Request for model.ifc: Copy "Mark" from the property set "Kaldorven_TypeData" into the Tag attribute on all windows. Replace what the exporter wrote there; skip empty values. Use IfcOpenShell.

First a look at what the model holds.

```python
import ifcopenshell
import ifcopenshell.util.element

model = ifcopenshell.open("model.ifc")
print(model.schema)
windows = model.by_type("IfcWindow")
print(len(windows), "windows")
for e in windows[:8]:
    source = ifcopenshell.util.element.get_pset(e, "Kaldorven_TypeData", "Mark")
    target = e.Tag
    print(e.id(), repr(source), repr(target), sep=" | ")
```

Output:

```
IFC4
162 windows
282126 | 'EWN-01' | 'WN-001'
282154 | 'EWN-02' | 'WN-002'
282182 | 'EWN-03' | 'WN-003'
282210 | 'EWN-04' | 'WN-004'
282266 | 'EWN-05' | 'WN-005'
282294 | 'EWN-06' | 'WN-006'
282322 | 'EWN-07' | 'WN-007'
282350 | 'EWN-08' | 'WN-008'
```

```python
import ifcopenshell
import ifcopenshell.util.element

model = ifcopenshell.open("model.ifc")

count = 0
for e in model.by_type("IfcWindow"):
    value = ifcopenshell.util.element.get_pset(e, "Kaldorven_TypeData", "Mark")
    current = e.Tag
    if not value or not value.strip() or current == value:
        continue
    e.Tag = value
    count += 1

print(count, "windows updated")

model.write("model_v2.ifc")
```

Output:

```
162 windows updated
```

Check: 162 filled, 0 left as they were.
